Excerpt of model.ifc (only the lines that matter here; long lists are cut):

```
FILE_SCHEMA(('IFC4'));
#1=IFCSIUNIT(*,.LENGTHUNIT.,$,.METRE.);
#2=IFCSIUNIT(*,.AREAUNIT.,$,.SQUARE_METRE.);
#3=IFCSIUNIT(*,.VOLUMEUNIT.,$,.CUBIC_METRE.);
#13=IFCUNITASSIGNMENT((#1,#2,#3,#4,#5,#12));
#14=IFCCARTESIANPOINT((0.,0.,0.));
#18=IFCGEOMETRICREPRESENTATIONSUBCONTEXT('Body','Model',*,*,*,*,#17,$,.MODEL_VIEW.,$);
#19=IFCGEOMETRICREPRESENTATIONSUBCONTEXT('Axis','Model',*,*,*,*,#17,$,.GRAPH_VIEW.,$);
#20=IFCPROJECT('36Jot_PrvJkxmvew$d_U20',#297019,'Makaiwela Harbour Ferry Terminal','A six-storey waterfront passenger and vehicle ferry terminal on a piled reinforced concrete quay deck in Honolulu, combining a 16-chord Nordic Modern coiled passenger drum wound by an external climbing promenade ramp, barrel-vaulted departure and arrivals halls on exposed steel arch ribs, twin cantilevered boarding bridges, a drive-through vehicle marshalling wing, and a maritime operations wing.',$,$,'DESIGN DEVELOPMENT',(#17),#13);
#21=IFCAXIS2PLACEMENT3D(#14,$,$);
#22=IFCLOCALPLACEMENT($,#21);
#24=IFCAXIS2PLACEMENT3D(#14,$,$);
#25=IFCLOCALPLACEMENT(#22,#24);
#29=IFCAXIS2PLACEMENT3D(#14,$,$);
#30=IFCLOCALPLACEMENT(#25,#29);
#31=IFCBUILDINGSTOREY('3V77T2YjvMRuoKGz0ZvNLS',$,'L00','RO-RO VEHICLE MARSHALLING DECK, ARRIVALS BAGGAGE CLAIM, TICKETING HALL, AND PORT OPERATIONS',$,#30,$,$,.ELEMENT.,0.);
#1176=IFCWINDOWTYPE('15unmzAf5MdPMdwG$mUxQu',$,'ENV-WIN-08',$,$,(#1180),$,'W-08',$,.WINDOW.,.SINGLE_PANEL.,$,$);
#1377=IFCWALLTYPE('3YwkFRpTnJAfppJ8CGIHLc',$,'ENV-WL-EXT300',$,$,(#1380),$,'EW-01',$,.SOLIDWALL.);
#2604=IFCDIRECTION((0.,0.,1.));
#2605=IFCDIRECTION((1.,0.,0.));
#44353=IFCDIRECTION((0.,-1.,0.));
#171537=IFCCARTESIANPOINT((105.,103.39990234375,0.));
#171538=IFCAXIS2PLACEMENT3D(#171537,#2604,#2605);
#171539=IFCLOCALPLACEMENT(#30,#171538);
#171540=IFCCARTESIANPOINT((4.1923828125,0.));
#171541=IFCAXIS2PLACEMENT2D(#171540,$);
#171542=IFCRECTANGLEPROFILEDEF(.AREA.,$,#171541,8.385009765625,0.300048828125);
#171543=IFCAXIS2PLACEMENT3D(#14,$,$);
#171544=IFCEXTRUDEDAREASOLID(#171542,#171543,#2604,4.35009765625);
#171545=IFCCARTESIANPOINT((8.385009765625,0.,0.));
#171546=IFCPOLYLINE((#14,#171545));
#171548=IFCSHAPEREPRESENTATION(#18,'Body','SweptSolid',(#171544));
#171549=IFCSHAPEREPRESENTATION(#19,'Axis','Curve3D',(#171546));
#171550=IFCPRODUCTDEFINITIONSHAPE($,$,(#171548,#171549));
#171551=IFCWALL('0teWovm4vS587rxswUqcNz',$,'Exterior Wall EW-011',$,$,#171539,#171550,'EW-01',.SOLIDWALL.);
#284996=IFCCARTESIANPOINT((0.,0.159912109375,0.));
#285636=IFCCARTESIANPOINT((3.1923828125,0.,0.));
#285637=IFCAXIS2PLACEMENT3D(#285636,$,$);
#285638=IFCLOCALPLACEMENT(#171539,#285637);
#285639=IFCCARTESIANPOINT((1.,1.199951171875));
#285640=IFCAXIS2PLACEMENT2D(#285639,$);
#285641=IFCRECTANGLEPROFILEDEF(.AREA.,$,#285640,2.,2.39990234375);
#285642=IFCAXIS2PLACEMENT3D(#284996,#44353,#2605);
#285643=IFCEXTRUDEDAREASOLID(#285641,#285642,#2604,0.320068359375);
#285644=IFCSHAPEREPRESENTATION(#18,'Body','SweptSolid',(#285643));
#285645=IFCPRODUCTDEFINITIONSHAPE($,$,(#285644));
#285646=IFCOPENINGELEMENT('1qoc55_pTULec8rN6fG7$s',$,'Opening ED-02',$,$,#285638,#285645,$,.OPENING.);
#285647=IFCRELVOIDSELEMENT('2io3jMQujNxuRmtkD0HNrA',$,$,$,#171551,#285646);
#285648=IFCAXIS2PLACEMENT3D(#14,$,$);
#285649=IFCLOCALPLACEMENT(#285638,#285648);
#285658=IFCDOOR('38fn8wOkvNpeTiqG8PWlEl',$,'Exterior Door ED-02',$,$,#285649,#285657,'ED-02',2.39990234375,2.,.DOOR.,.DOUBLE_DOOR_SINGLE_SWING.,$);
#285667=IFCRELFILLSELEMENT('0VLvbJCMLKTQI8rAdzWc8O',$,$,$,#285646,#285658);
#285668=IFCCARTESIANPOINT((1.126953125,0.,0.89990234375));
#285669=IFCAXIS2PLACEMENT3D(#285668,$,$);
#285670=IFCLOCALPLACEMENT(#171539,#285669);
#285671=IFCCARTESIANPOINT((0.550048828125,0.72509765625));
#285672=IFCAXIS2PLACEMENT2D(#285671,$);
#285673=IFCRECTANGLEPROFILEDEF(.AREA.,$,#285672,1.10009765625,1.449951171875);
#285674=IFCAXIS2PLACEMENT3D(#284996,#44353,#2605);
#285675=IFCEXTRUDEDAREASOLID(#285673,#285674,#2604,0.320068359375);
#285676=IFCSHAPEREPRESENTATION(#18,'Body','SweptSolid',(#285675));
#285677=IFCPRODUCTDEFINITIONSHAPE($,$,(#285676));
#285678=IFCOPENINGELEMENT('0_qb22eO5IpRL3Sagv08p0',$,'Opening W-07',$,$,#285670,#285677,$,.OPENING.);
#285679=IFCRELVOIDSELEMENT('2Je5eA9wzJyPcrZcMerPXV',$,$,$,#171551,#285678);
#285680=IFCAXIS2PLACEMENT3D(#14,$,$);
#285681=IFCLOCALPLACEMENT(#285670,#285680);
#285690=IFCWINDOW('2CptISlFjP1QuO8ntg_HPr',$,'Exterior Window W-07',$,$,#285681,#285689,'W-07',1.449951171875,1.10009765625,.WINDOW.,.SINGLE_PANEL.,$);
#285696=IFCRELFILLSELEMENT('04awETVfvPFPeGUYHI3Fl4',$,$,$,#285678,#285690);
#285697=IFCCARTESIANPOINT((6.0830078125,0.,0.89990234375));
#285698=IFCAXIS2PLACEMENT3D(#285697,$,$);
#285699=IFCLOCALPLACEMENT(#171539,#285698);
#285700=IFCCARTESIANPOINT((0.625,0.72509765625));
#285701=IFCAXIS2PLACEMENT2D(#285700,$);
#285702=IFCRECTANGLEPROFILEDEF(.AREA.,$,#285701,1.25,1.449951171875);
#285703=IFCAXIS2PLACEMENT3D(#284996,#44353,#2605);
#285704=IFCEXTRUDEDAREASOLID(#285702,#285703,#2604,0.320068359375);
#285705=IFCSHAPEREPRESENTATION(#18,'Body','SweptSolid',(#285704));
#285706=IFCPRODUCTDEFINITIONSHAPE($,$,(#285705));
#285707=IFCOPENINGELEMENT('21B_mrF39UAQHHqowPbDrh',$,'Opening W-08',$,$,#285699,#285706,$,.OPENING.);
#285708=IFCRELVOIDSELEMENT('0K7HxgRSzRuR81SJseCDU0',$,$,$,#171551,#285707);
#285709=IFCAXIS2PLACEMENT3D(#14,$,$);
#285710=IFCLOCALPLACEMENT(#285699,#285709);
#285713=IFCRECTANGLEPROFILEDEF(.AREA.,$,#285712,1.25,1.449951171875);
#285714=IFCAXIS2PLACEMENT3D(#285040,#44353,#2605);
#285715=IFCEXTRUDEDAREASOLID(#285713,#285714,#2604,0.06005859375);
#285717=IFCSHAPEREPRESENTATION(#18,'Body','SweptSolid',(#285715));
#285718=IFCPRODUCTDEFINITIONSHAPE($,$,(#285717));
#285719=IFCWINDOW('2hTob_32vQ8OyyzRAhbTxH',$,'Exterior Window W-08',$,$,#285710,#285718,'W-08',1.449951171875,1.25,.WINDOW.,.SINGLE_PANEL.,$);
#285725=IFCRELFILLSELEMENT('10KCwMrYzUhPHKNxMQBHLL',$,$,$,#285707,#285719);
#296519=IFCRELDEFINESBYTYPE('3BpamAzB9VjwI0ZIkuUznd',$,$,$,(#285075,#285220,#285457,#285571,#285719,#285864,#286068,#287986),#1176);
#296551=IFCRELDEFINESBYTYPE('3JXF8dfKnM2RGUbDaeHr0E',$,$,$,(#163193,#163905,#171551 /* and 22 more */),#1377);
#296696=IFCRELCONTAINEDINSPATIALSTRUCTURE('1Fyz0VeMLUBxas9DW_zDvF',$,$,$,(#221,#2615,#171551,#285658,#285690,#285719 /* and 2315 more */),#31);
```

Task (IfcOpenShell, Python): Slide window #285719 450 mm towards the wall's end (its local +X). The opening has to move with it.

```python
import ifcopenshell
import ifcopenshell.api.geometry
import ifcopenshell.util.placement
import ifcopenshell.util.unit

model = ifcopenshell.open("model.ifc")
unit_scale = ifcopenshell.util.unit.calculate_unit_scale(model)

window = model.by_id(285719)
opening = window.FillsVoids[0].RelatingOpeningElement
wall = opening.VoidsElements[0].RelatingBuildingElement

wall_matrix = ifcopenshell.util.placement.get_local_placement(wall.ObjectPlacement)
shift = wall_matrix[:3, 0] * 0.45 / unit_scale
before = ifcopenshell.util.placement.get_local_placement(window.ObjectPlacement)[:3, 3].copy()

# The window is placed relative to its opening, so it follows when the opening moves.
matrix = ifcopenshell.util.placement.get_local_placement(opening.ObjectPlacement)
matrix[:3, 3] += shift
ifcopenshell.api.geometry.edit_object_placement(
    model, product=opening, matrix=matrix, is_si=False, should_transform_children=True
)

after = ifcopenshell.util.placement.get_local_placement(window.ObjectPlacement)[:3, 3]
print("window moved by", (after - before).round(3) + 0.0)

model.write("model_v2.ifc")
```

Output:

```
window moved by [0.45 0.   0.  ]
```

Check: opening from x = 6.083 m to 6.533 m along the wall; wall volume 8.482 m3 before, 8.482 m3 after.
